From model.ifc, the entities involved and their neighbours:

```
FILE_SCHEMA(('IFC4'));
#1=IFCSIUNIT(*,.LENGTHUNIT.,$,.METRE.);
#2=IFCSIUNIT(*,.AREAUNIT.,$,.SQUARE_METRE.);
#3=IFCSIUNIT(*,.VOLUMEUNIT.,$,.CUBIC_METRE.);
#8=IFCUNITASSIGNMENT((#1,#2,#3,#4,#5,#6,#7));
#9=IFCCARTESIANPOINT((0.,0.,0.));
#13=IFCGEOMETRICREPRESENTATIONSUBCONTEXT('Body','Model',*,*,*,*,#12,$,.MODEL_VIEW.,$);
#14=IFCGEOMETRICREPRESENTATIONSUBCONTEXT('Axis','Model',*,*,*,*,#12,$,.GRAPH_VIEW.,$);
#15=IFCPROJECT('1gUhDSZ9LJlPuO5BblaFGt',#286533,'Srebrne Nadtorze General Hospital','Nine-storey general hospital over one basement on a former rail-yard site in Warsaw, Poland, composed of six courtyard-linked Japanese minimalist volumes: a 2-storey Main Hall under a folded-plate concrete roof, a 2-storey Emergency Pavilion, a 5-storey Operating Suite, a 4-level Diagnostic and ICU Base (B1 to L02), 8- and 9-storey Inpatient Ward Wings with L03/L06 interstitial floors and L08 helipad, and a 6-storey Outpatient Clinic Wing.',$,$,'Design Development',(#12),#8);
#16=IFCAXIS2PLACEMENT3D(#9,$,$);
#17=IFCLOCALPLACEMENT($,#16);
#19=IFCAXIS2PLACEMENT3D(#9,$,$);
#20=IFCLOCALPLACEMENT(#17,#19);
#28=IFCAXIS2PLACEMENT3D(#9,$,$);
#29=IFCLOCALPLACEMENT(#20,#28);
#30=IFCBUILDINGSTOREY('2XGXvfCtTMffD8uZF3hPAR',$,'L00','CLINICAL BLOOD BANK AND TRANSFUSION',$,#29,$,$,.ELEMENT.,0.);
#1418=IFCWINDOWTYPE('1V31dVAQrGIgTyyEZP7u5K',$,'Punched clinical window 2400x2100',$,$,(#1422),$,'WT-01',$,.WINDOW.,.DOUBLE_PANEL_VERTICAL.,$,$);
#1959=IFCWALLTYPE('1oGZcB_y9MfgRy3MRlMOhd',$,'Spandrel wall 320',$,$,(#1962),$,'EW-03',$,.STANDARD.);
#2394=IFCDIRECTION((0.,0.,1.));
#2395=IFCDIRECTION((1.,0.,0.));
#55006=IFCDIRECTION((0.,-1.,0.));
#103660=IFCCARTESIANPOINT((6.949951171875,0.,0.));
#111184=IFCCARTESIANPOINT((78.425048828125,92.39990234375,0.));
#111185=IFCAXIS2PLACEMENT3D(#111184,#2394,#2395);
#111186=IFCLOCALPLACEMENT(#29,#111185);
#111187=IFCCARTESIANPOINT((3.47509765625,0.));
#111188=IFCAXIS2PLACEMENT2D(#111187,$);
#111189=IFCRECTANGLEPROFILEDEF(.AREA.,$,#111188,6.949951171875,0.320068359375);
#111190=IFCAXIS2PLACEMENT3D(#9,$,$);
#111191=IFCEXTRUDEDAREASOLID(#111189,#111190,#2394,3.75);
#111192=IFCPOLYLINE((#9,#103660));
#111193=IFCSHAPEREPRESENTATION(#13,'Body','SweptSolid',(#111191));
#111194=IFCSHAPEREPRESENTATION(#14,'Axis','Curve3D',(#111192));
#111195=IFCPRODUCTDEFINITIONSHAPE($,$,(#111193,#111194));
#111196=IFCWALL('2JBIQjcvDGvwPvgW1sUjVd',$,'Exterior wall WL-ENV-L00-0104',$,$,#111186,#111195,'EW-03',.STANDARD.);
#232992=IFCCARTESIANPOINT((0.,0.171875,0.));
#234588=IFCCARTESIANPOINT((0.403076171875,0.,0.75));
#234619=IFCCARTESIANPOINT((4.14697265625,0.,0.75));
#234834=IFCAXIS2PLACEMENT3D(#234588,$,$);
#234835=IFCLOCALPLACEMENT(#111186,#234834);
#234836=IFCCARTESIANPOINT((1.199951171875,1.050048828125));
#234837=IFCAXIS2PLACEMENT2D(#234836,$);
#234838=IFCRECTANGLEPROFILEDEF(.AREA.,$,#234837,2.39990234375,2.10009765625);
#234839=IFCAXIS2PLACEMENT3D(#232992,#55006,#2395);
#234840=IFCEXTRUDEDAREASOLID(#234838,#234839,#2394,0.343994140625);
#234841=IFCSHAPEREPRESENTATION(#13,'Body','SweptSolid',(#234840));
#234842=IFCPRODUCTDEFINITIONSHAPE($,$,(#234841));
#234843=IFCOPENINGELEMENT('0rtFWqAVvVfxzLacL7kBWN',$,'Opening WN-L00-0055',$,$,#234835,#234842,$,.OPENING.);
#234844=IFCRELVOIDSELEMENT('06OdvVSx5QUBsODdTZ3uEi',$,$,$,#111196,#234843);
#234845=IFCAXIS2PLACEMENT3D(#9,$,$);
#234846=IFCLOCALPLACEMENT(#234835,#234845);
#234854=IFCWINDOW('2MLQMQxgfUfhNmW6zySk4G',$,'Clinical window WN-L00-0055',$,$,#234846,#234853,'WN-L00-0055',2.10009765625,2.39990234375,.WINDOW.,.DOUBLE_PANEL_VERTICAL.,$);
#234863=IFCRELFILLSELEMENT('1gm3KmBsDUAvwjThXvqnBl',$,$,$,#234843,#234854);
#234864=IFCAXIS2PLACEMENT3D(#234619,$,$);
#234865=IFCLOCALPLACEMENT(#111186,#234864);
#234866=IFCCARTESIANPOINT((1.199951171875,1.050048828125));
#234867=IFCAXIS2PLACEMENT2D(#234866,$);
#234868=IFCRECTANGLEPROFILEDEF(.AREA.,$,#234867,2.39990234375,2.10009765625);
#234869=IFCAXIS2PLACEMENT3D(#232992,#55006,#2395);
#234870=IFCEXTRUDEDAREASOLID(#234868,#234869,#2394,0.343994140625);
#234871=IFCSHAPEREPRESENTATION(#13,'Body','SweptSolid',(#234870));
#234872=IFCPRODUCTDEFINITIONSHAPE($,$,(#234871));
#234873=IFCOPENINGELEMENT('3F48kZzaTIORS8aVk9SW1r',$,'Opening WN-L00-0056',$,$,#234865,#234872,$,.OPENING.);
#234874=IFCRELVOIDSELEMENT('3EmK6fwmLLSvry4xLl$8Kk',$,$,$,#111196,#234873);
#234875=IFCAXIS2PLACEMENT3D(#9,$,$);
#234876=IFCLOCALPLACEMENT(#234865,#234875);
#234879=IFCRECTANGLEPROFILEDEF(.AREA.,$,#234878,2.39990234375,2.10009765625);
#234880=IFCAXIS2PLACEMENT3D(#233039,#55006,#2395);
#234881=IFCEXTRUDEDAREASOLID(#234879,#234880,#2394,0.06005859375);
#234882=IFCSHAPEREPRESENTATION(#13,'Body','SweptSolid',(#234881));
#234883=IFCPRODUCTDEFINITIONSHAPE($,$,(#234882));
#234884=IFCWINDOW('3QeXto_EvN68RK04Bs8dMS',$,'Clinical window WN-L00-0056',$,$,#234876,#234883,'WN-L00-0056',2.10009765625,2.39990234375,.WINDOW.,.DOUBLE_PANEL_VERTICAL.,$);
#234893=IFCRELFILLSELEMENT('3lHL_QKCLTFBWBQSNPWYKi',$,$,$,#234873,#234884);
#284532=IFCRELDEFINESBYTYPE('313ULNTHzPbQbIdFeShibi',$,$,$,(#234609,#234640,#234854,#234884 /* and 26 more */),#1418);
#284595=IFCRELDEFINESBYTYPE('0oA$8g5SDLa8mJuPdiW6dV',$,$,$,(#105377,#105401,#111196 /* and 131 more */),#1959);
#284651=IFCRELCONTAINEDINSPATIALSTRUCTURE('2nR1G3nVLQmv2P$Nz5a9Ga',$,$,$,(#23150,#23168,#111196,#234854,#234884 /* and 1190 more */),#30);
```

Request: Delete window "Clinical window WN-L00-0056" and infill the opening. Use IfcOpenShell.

```python
import ifcopenshell
import ifcopenshell.api.feature
import ifcopenshell.api.root
import ifcopenshell.geom
import ifcopenshell.util.shape

model = ifcopenshell.open("model.ifc")
settings = ifcopenshell.geom.settings()


def volume(element):
    """Net volume in cubic metres, openings subtracted."""
    shape = ifcopenshell.geom.create_shape(settings, element)
    return ifcopenshell.util.shape.get_volume(shape.geometry)


window = model.by_id(234884)
opening = window.FillsVoids[0].RelatingOpeningElement
wall = opening.VoidsElements[0].RelatingBuildingElement
before = volume(wall)

ifcopenshell.api.root.remove_product(model, product=window)
ifcopenshell.api.feature.remove_feature(model, feature=opening)

after = volume(wall)

print(f"wall volume {before:.3f} -> {after:.3f} m3")

model.write("model_rev.ifc")
```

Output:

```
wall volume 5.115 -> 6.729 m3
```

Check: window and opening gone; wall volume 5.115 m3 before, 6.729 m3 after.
